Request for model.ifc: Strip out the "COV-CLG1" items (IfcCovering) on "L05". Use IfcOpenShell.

First a look at what the model holds.

```python
import ifcopenshell
import ifcopenshell.util.element

model = ifcopenshell.open("model.ifc")
print(model.schema)
storey = next(s for s in model.by_type("IfcBuildingStorey") if s.Name == "L05")
coverings = [e for e in ifcopenshell.util.element.get_decomposition(storey) if e.is_a("IfcCovering")]
seen = {}
for e in coverings:
    element_type = ifcopenshell.util.element.get_type(e)
    name = element_type.Name if element_type not in (None, e) else None
    seen[name] = seen.get(name, 0) + 1
for name, count in sorted(seen.items(), key=str):
    print(count, "x", name)
```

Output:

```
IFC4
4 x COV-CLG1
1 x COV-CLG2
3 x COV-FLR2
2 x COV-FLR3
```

```python
import ifcopenshell
import ifcopenshell.api.root
import ifcopenshell.util.element

model = ifcopenshell.open("model.ifc")

storey = next(s for s in model.by_type("IfcBuildingStorey") if s.Name == "L05")
coverings = [e for e in ifcopenshell.util.element.get_decomposition(storey) if e.is_a("IfcCovering")]
targets = [e for e in coverings if (t := ifcopenshell.util.element.get_type(e)) not in (None, e) and t.Name == "COV-CLG1"]

for e in targets:
    ifcopenshell.api.root.remove_product(model, product=e)
print(len(targets), "removed")

model.write("model_updated.ifc")
```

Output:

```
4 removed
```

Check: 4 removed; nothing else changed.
